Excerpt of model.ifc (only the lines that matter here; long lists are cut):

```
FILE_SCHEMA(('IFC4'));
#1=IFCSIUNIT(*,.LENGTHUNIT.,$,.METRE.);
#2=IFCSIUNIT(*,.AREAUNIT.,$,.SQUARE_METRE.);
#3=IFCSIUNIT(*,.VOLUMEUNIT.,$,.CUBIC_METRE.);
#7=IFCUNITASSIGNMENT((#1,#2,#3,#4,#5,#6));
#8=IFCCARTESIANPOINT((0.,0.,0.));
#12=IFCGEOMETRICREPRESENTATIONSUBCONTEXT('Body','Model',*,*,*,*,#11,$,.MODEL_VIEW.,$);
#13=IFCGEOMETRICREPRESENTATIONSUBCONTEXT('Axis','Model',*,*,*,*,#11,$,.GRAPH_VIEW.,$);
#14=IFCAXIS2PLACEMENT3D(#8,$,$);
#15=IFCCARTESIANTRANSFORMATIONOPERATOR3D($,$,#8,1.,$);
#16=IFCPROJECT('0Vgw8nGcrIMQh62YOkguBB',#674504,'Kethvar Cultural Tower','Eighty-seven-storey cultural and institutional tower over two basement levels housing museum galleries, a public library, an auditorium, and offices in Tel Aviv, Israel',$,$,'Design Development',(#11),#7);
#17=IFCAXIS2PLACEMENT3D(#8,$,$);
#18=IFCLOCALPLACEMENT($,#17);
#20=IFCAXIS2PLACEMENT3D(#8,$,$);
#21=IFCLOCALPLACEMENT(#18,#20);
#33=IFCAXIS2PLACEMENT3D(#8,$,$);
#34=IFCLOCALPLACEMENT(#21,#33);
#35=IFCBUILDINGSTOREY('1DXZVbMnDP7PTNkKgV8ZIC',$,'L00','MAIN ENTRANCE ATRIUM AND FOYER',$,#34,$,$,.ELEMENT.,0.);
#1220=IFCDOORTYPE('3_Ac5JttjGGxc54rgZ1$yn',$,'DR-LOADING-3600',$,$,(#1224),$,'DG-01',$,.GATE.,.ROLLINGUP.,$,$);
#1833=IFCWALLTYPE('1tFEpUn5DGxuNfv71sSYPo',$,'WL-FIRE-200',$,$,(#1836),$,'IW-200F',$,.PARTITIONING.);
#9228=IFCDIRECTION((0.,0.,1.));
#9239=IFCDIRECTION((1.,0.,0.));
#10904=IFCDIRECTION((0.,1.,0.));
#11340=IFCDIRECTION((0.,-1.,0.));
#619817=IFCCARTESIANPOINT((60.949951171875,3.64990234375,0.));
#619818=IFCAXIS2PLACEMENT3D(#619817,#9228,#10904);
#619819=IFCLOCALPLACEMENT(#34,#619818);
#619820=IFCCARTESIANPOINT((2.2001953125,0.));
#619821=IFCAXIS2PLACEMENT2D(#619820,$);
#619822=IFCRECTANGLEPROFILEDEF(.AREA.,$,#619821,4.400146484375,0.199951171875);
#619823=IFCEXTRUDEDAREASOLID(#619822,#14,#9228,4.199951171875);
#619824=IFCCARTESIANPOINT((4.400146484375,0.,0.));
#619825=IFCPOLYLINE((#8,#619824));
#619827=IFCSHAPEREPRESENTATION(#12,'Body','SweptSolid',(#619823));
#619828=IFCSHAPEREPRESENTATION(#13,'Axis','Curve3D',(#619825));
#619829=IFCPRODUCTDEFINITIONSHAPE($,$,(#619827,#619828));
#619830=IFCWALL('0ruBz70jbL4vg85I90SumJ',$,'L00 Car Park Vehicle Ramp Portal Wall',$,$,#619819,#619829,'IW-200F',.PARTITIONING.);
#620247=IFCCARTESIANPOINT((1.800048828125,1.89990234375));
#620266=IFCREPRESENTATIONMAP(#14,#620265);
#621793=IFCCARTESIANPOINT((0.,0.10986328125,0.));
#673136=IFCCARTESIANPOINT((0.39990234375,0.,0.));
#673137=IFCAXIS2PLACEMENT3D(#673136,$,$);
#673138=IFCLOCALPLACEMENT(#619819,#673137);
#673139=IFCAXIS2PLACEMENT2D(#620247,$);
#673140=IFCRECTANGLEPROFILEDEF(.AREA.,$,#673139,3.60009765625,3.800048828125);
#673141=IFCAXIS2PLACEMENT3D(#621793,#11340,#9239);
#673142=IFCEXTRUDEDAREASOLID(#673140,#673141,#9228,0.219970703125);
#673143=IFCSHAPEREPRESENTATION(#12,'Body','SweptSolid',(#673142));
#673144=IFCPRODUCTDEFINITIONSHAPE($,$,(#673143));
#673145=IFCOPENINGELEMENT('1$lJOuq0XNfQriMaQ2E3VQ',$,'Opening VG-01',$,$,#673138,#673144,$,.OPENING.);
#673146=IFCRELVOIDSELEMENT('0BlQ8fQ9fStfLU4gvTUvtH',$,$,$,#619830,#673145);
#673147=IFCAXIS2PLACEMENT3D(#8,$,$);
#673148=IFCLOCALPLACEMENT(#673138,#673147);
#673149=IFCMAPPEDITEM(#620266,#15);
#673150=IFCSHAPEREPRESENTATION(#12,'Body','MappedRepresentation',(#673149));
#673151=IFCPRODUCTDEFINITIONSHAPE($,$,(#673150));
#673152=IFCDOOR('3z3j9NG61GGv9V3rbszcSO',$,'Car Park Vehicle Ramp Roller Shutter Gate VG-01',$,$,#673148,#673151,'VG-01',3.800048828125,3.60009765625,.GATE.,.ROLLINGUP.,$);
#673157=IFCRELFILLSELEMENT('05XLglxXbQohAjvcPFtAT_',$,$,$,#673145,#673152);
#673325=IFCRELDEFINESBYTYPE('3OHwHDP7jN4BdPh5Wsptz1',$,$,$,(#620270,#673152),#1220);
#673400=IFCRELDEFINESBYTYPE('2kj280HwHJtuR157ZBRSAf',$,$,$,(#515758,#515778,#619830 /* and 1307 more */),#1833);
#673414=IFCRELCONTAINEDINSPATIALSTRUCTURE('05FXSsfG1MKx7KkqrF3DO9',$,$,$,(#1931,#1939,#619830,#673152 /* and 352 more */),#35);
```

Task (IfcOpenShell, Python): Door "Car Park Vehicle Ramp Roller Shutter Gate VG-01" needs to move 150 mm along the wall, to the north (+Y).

```python
import ifcopenshell
import ifcopenshell.api.geometry
import ifcopenshell.util.placement

model = ifcopenshell.open("model.ifc")

door = model.by_id(673152)
opening = door.FillsVoids[0].RelatingOpeningElement
wall = opening.VoidsElements[0].RelatingBuildingElement

wall_matrix = ifcopenshell.util.placement.get_local_placement(wall.ObjectPlacement)
shift = wall_matrix[:3, 0] * 0.15
before = ifcopenshell.util.placement.get_local_placement(door.ObjectPlacement)[:3, 3].copy()

# The door is placed relative to its opening, so it follows when the opening moves.
matrix = ifcopenshell.util.placement.get_local_placement(opening.ObjectPlacement)
matrix[:3, 3] += shift
ifcopenshell.api.geometry.edit_object_placement(
    model, product=opening, matrix=matrix, is_si=False, should_transform_children=True
)

after = ifcopenshell.util.placement.get_local_placement(door.ObjectPlacement)[:3, 3]
print("door moved by", (after - before).round(3) + 0.0)

model.write("model-out.ifc")
```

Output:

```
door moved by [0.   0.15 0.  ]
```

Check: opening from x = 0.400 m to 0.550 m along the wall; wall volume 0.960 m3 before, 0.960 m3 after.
